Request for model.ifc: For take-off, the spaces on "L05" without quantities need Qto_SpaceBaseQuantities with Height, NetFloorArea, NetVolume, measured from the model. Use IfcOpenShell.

First a look at what the model holds.

```python
import ifcopenshell
import ifcopenshell.util.element
import ifcopenshell.util.unit

model = ifcopenshell.open("model.ifc")
print(model.schema)
for unit_type in ("LENGTHUNIT", "AREAUNIT", "VOLUMEUNIT"):
    print(unit_type, ifcopenshell.util.unit.calculate_unit_scale(model, unit_type))
storey = next(s for s in model.by_type("IfcBuildingStorey") if s.Name == "L05")
spaces = [e for e in ifcopenshell.util.element.get_decomposition(storey) if e.is_a("IfcSpace")]
for e in sorted(spaces, key=lambda e: e.id()):
    print(e.id(), e.is_a(), e.Name, list(ifcopenshell.util.element.get_psets(e, qtos_only=True)), sep=" | ")
```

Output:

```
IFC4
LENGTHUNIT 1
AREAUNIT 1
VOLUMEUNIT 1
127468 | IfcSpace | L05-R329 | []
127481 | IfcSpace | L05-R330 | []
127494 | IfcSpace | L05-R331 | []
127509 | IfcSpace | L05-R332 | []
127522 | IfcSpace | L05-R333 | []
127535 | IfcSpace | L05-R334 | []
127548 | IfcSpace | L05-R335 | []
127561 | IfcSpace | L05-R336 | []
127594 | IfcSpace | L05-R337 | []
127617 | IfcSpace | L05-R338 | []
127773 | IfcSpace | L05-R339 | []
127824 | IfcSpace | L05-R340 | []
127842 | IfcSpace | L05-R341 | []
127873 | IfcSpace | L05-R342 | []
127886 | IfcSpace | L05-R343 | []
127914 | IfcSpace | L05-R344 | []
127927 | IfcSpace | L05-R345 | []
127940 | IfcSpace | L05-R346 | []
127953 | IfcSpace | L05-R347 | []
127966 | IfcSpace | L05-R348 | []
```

```python
import ifcopenshell
import ifcopenshell.api.pset
import ifcopenshell.geom
import ifcopenshell.util.element
import ifcopenshell.util.shape
import ifcopenshell.util.unit

model = ifcopenshell.open("model.ifc")
unit_scale = ifcopenshell.util.unit.calculate_unit_scale(model)
area_scale = ifcopenshell.util.unit.calculate_unit_scale(model, "AREAUNIT")
volume_scale = ifcopenshell.util.unit.calculate_unit_scale(model, "VOLUMEUNIT")
settings = ifcopenshell.geom.settings()

storey = next(s for s in model.by_type("IfcBuildingStorey") if s.Name == "L05")
spaces = [e for e in ifcopenshell.util.element.get_decomposition(storey) if e.is_a("IfcSpace")]

for e in sorted(spaces, key=lambda e: e.id()):
    if ifcopenshell.util.element.get_psets(e, qtos_only=True, should_inherit=False):
        continue
    # Geometry comes back in metres, in the element's own axes.
    shape = ifcopenshell.geom.create_shape(settings, e)
    values = {
        "Height": ifcopenshell.util.shape.get_z(shape.geometry) / unit_scale,
        "NetFloorArea": ifcopenshell.util.shape.get_footprint_area(shape.geometry) / area_scale,
        "NetVolume": ifcopenshell.util.shape.get_volume(shape.geometry) / volume_scale,
    }
    qto = ifcopenshell.api.pset.add_qto(model, product=e, name="Qto_SpaceBaseQuantities")
    ifcopenshell.api.pset.edit_qto(model, qto=qto, properties=values)
    print(e.id(), {k: round(v, 3) for k, v in values.items()})

model.write("model-out.ifc")
```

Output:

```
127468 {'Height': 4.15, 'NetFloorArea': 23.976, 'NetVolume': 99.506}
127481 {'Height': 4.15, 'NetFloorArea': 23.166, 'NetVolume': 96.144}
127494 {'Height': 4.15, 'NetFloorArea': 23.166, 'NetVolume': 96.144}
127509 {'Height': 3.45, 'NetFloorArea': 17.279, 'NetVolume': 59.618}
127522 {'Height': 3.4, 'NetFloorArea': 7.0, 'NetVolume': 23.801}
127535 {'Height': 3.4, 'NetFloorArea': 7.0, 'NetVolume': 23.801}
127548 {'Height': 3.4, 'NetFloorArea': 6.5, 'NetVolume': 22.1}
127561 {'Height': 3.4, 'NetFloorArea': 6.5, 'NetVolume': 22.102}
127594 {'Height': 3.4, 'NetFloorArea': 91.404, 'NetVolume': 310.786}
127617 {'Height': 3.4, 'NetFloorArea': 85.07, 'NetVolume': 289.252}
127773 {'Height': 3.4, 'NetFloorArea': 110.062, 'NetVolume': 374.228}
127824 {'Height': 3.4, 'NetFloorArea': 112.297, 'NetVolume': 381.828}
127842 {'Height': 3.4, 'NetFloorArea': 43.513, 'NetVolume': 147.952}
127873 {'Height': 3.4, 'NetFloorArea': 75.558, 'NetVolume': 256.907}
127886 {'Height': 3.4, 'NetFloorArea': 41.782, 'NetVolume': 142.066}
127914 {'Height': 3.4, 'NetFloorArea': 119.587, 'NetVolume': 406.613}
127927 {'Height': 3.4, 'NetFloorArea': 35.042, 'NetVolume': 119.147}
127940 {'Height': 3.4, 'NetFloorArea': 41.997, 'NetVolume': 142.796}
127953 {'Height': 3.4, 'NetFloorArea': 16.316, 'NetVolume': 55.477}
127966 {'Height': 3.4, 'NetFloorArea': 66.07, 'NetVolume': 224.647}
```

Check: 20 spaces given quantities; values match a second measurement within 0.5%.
